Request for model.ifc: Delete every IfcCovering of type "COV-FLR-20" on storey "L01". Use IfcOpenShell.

First a look at what the model holds.

```python
import ifcopenshell
import ifcopenshell.util.element

model = ifcopenshell.open("model.ifc")
print(model.schema)
storey = next(s for s in model.by_type("IfcBuildingStorey") if s.Name == "L01")
coverings = [e for e in ifcopenshell.util.element.get_decomposition(storey) if e.is_a("IfcCovering")]
seen = {}
for e in coverings:
    element_type = ifcopenshell.util.element.get_type(e)
    name = element_type.Name if element_type not in (None, e) else None
    seen[name] = seen.get(name, 0) + 1
for name, count in sorted(seen.items(), key=str):
    print(count, "x", name)
```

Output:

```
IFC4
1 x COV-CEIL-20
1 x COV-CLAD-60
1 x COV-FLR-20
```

```python
import ifcopenshell
import ifcopenshell.api.root
import ifcopenshell.util.element

model = ifcopenshell.open("model.ifc")

storey = next(s for s in model.by_type("IfcBuildingStorey") if s.Name == "L01")
coverings = [e for e in ifcopenshell.util.element.get_decomposition(storey) if e.is_a("IfcCovering")]
targets = [e for e in coverings if (t := ifcopenshell.util.element.get_type(e)) not in (None, e) and t.Name == "COV-FLR-20"]

for e in targets:
    ifcopenshell.api.root.remove_product(model, product=e)
print(len(targets), "removed")

model.write("model-out.ifc")
```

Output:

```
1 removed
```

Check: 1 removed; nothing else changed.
